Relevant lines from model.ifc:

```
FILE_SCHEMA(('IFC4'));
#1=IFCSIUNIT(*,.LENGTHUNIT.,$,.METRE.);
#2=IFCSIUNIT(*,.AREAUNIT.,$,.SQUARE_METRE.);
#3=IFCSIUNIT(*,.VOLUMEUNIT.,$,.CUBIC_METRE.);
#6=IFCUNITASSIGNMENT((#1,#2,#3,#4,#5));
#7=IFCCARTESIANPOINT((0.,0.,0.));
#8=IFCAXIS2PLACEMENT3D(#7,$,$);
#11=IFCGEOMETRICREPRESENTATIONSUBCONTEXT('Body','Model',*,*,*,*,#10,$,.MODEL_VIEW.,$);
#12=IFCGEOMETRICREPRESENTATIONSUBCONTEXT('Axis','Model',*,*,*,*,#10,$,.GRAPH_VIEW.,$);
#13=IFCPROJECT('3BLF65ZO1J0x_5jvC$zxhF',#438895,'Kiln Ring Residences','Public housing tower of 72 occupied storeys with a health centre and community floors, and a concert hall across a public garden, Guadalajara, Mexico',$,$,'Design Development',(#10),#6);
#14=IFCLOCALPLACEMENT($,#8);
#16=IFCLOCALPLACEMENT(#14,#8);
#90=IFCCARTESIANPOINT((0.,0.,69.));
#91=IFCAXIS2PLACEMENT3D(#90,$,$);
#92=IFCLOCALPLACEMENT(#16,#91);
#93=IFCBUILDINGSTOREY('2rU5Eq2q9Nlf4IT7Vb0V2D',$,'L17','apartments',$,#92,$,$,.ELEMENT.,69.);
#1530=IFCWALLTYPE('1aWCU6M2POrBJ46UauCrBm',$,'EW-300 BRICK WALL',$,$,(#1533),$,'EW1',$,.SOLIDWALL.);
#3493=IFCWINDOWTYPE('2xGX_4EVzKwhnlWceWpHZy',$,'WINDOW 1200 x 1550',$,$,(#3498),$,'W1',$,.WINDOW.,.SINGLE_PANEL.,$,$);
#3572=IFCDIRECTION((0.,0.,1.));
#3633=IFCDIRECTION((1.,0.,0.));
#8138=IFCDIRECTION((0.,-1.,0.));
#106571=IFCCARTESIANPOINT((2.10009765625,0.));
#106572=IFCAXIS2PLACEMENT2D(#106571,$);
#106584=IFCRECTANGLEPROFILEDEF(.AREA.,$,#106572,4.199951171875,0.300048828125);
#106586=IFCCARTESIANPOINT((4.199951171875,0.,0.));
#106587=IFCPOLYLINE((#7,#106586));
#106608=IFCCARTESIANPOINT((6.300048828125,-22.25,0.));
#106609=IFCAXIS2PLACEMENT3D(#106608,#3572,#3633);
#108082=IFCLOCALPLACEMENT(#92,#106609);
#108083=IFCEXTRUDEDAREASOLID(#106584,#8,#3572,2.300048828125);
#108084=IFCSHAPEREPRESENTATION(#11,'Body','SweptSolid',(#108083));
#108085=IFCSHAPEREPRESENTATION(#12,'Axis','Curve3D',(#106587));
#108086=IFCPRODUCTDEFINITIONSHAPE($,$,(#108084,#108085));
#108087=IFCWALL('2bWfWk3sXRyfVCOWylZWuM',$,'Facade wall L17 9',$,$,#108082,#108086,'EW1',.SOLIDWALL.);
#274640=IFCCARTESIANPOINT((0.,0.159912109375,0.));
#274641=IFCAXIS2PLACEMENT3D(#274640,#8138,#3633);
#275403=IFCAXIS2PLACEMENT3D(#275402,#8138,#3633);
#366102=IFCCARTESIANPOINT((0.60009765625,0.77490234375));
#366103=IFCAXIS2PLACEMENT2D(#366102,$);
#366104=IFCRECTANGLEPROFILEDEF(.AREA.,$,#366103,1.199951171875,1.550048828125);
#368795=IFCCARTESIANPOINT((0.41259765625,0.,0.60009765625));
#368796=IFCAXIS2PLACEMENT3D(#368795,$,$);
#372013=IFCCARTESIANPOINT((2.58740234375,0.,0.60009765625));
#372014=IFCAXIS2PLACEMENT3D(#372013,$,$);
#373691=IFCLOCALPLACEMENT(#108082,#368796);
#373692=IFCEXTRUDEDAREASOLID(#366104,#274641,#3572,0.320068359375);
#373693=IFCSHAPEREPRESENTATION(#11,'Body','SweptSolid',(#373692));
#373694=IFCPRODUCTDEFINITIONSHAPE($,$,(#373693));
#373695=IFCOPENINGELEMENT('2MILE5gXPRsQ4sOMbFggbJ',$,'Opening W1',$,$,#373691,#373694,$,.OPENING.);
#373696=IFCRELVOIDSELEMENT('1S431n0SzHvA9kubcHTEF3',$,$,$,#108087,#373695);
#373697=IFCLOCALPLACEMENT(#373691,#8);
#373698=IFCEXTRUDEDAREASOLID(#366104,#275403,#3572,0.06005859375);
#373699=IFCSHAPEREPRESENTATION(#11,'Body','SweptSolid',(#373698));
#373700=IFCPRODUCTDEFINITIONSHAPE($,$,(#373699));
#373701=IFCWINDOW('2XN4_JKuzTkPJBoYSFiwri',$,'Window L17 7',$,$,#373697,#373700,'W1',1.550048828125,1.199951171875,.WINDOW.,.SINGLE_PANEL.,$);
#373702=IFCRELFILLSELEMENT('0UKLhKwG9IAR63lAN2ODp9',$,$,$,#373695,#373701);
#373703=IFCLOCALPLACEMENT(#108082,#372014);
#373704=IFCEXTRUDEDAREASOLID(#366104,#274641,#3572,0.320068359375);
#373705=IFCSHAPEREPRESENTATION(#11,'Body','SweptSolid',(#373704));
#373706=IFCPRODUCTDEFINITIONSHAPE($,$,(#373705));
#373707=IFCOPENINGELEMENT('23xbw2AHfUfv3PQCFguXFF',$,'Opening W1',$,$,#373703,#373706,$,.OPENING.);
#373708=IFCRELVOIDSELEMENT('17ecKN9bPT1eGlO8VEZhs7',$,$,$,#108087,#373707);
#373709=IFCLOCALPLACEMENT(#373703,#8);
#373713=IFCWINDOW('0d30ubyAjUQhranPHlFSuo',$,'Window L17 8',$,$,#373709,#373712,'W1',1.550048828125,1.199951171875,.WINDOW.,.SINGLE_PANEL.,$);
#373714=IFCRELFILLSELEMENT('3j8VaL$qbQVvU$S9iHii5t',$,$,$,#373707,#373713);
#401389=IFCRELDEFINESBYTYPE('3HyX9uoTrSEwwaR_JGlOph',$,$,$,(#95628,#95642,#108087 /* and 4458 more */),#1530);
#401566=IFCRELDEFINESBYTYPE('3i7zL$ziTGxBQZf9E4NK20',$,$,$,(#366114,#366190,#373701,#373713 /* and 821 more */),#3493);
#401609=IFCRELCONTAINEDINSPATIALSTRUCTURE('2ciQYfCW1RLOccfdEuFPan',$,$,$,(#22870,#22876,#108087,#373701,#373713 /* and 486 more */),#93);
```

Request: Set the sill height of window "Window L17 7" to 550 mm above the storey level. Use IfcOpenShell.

```python
import numpy as np
import ifcopenshell
import ifcopenshell.api.geometry
import ifcopenshell.geom
import ifcopenshell.util.element
import ifcopenshell.util.placement
import ifcopenshell.util.shape
import ifcopenshell.util.unit

model = ifcopenshell.open("model.ifc")
unit_scale = ifcopenshell.util.unit.calculate_unit_scale(model)

window = model.by_guid("2XN4_JKuzTkPJBoYSFiwri")
opening = window.FillsVoids[0].RelatingOpeningElement
storey = ifcopenshell.util.element.get_container(window, ifc_class="IfcBuildingStorey")
level = ifcopenshell.util.placement.get_local_placement(storey.ObjectPlacement)[2, 3]

# The opening's origin need not be at the sill, so measure its lowest point.
shape = ifcopenshell.geom.create_shape(ifcopenshell.geom.settings(), opening)
bottom = ifcopenshell.util.shape.get_shape_bottom_elevation(shape, shape.geometry) / unit_scale
dz = level + 0.55 / unit_scale - bottom

shift = np.array([0.0, 0.0, dz])
# The window is placed relative to its opening, so it follows when the opening moves.
matrix = ifcopenshell.util.placement.get_local_placement(opening.ObjectPlacement)
matrix[:3, 3] += shift
ifcopenshell.api.geometry.edit_object_placement(
    model, product=opening, matrix=matrix, is_si=False, should_transform_children=True
)

print(f"moved by {dz * unit_scale:+.3f} m")

model.write("model_updated.ifc")
```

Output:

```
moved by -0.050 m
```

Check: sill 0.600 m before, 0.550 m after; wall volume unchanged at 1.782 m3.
